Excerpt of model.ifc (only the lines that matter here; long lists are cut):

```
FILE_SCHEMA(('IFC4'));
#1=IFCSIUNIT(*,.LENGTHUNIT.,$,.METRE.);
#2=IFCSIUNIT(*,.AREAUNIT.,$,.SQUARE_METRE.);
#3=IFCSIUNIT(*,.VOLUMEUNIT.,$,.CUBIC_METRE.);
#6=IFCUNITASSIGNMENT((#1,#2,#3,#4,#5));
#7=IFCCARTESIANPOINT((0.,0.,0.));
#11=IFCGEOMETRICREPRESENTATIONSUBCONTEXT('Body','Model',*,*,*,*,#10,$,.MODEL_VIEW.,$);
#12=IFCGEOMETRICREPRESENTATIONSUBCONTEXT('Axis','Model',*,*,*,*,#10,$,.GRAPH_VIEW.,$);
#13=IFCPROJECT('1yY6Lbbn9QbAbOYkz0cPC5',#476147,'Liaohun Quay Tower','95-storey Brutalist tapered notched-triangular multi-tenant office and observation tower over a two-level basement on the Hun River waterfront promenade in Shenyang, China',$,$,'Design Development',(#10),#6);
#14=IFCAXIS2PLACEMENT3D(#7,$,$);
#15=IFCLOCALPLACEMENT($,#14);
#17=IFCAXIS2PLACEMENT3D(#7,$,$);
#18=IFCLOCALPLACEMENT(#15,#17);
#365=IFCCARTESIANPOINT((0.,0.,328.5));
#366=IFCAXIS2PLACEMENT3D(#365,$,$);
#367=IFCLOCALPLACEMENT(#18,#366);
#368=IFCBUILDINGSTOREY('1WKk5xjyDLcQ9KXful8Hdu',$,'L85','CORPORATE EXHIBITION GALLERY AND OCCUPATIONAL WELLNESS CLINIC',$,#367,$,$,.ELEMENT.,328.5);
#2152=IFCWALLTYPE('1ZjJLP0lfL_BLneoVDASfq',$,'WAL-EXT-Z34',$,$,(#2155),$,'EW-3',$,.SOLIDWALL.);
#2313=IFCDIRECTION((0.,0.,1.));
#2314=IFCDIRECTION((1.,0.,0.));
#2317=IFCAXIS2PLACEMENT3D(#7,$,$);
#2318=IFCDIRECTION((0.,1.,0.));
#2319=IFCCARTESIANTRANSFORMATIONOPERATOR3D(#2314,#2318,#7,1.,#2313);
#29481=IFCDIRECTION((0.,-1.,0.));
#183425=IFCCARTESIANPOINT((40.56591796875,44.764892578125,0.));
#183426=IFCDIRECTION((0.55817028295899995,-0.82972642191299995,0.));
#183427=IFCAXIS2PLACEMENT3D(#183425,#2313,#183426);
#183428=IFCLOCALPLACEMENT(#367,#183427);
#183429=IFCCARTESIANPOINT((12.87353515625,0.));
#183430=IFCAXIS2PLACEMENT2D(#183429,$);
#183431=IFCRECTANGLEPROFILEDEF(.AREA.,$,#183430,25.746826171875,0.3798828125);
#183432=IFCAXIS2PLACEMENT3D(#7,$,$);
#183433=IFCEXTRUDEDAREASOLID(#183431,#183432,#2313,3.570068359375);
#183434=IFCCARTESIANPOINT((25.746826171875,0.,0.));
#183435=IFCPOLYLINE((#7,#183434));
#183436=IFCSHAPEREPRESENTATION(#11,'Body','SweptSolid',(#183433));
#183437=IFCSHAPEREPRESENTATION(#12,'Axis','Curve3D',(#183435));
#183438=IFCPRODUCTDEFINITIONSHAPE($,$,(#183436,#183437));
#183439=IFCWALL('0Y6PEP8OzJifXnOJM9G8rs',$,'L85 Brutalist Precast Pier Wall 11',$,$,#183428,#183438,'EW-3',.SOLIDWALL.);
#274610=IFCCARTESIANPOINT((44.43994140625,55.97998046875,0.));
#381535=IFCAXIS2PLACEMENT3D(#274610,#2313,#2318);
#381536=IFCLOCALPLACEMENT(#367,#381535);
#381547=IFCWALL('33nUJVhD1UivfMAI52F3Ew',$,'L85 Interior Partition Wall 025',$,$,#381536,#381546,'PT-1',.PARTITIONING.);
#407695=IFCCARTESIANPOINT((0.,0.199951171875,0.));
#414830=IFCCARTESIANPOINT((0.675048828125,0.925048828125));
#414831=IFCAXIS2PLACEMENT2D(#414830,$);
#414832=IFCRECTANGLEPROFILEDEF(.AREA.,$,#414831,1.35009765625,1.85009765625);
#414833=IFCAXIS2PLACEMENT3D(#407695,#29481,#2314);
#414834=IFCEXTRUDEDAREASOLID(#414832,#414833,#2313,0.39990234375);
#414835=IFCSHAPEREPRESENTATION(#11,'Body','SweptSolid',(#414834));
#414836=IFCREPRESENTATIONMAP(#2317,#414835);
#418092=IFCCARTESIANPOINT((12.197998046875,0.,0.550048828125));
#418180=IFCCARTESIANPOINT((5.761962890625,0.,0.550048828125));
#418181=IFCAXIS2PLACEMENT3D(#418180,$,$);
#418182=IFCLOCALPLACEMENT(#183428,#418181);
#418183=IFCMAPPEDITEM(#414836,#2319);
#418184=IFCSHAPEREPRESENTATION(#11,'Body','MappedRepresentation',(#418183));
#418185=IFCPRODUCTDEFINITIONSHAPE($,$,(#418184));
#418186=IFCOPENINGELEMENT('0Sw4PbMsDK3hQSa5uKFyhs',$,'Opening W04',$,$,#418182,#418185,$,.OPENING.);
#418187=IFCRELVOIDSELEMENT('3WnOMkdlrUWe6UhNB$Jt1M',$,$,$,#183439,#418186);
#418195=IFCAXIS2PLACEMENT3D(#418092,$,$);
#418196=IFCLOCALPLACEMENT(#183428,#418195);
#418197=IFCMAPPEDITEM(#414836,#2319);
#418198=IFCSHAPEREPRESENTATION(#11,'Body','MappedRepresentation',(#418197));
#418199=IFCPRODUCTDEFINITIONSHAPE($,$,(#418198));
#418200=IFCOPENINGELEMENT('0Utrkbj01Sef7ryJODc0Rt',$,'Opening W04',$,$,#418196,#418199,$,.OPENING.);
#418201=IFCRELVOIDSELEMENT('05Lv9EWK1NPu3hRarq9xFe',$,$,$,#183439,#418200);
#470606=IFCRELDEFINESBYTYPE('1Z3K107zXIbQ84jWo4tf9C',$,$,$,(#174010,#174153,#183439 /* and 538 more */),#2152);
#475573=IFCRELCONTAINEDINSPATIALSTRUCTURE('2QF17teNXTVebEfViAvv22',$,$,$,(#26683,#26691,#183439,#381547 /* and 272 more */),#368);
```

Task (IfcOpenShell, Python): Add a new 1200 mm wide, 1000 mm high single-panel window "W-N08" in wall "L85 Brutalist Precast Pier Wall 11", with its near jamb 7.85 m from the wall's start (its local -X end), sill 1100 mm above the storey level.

```python
import numpy as np
import ifcopenshell
import ifcopenshell.api.feature
import ifcopenshell.api.geometry
import ifcopenshell.api.root
import ifcopenshell.api.spatial
import ifcopenshell.geom
import ifcopenshell.util.element
import ifcopenshell.util.placement
import ifcopenshell.util.representation
import ifcopenshell.util.shape
import ifcopenshell.util.unit

model = ifcopenshell.open("model.ifc")
unit_scale = ifcopenshell.util.unit.calculate_unit_scale(model)
settings = ifcopenshell.geom.settings()


def volume(element):
    """Net volume in cubic metres, openings subtracted."""
    shape = ifcopenshell.geom.create_shape(settings, element)
    return ifcopenshell.util.shape.get_volume(shape.geometry)


wall = model.by_guid("0Y6PEP8OzJifXnOJM9G8rs")
storey = ifcopenshell.util.element.get_container(wall, ifc_class="IfcBuildingStorey")
context = ifcopenshell.util.representation.get_context(model, "Model", "Body", "MODEL_VIEW")
before = volume(wall)

width, height, from_end, sill = 1.2, 1, 7.85, 1.1  # metres

# The wall runs along its own X axis, and the end named is its -X end.
wall_shape = ifcopenshell.geom.create_shape(settings, wall)
x, y, z = ifcopenshell.util.shape.get_vertices(wall_shape.geometry).T
start = x.min() + from_end
face, thickness = float(y.min()), float(y.max() - y.min())
wall_matrix = ifcopenshell.util.placement.get_local_placement(wall.ObjectPlacement)
level = ifcopenshell.util.placement.get_local_placement(storey.ObjectPlacement)[2, 3]


def in_wall(x, y):
    """Placement at x, y metres in the wall's axes, at sill height."""
    matrix = wall_matrix.copy()
    matrix[:, 3] = wall_matrix @ np.array([x / unit_scale, y / unit_scale, 0.0, 1.0])
    matrix[2, 3] = level + sill / unit_scale
    return matrix


# Opening: a box that overshoots both wall faces by 50 mm.
opening = ifcopenshell.api.root.create_entity(model, ifc_class="IfcOpeningElement", predefined_type="OPENING")
box = ifcopenshell.api.geometry.add_wall_representation(
    model, context=context, length=width, height=height, thickness=thickness + 0.1
)
ifcopenshell.api.geometry.assign_representation(model, product=opening, representation=box)
ifcopenshell.api.geometry.edit_object_placement(model, product=opening, matrix=in_wall(start, face - 0.05), is_si=False)
ifcopenshell.api.feature.add_feature(model, feature=opening, element=wall)

window = ifcopenshell.api.root.create_entity(model, ifc_class="IfcWindow", name="W-N08", predefined_type="WINDOW")
window.OverallWidth, window.OverallHeight = width / unit_scale, height / unit_scale
window.PartitioningType = "SINGLE_PANEL"
body = ifcopenshell.api.geometry.add_window_representation(
    model,
    context=context,
    overall_width=window.OverallWidth,
    overall_height=window.OverallHeight,
    partition_type="SINGLE_PANEL",
)
ifcopenshell.api.geometry.assign_representation(model, product=window, representation=body)
ifcopenshell.api.spatial.assign_container(model, products=[window], relating_structure=storey)
ifcopenshell.api.feature.add_filling(model, opening=opening, element=window)

# Centre the window in the wall's thickness.
ifcopenshell.api.geometry.edit_object_placement(model, product=window, matrix=in_wall(start, face), is_si=False)
window_shape = ifcopenshell.geom.create_shape(settings, window)
depth = ifcopenshell.util.shape.get_vertices(window_shape.geometry)[:, 1]
offset = face + thickness / 2 - (depth.min() + depth.max()) / 2
ifcopenshell.api.geometry.edit_object_placement(model, product=window, matrix=in_wall(start, offset), is_si=False)

after = volume(wall)

print(f"wall volume {before:.3f} -> {after:.3f} m3")

model.write("model_edited.ifc")
```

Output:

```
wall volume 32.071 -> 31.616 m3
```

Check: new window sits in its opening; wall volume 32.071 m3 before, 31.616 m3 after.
